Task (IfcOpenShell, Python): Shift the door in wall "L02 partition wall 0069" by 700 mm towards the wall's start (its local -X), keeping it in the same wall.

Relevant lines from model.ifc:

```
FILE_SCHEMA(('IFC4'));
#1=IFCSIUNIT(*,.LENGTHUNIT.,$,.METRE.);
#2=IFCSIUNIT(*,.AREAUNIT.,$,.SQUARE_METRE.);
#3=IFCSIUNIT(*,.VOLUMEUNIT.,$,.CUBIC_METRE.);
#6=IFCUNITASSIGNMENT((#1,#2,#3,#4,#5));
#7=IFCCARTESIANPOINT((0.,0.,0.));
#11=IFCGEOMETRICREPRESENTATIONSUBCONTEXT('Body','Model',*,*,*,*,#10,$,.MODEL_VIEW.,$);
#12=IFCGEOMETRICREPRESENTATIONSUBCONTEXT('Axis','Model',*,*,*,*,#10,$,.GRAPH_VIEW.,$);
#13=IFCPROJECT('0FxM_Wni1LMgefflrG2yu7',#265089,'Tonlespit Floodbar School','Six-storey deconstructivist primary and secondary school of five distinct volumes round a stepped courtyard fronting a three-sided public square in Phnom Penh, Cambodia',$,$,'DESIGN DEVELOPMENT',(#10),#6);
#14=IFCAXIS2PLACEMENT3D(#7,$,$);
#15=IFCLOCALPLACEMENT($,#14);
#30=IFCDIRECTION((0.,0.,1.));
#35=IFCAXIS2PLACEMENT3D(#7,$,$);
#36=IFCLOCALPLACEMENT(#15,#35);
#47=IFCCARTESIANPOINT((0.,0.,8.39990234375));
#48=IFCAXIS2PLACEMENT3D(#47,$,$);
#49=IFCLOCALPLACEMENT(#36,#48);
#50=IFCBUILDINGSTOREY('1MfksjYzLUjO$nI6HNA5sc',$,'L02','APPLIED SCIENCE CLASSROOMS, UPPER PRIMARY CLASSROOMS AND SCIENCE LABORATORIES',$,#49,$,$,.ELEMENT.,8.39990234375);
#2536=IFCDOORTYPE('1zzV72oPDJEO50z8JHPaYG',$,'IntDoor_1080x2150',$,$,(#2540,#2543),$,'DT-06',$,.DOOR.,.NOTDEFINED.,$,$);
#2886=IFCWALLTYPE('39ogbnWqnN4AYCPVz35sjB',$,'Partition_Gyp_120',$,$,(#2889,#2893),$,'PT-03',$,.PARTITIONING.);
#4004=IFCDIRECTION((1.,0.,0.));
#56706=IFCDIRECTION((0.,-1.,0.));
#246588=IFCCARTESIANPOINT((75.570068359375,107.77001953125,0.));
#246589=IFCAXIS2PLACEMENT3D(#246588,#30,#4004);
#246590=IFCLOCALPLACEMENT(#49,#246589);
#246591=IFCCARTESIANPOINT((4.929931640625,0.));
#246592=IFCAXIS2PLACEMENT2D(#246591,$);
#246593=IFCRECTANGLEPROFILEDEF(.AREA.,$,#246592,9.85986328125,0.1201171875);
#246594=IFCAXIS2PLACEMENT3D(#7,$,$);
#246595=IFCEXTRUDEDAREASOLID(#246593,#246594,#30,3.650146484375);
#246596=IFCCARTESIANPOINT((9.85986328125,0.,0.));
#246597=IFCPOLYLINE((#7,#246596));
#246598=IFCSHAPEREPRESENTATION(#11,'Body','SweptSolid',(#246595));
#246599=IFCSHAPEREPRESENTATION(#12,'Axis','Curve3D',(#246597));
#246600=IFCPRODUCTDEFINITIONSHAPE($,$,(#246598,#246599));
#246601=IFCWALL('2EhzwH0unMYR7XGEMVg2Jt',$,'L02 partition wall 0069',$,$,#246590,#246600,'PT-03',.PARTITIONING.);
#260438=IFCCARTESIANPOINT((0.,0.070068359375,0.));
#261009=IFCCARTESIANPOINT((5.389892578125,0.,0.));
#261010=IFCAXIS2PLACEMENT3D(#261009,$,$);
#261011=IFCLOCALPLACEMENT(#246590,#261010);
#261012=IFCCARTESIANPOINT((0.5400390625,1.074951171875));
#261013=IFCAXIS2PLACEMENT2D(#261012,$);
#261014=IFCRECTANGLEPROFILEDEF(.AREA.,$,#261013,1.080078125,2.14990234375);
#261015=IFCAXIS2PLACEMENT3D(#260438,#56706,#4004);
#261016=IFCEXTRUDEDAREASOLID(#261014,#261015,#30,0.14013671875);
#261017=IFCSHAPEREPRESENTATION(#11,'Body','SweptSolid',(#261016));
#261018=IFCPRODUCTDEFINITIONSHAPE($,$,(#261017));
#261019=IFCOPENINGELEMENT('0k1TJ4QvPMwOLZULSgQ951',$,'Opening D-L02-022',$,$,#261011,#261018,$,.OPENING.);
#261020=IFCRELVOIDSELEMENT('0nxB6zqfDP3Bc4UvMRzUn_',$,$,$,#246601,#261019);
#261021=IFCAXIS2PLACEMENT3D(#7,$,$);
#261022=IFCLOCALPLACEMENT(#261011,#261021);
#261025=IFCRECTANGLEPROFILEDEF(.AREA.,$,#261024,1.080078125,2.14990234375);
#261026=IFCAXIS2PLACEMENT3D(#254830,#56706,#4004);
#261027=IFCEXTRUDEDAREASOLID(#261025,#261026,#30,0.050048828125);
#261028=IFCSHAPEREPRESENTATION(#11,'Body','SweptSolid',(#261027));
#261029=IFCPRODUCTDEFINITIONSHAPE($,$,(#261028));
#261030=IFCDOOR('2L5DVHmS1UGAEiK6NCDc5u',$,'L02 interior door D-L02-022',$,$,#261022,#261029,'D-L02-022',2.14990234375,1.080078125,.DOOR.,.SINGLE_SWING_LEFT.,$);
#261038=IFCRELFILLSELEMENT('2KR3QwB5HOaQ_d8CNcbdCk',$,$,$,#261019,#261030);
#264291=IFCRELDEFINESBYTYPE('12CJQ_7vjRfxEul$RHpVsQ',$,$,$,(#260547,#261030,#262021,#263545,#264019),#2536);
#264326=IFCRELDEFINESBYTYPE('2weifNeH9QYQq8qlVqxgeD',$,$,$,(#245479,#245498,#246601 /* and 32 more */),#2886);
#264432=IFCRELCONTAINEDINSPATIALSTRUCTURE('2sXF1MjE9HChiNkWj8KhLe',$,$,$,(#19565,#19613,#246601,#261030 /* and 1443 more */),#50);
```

```python
import ifcopenshell
import ifcopenshell.api.geometry
import ifcopenshell.util.placement
import ifcopenshell.util.unit

model = ifcopenshell.open("model.ifc")
unit_scale = ifcopenshell.util.unit.calculate_unit_scale(model)

door = model.by_guid("2L5DVHmS1UGAEiK6NCDc5u")
opening = door.FillsVoids[0].RelatingOpeningElement
wall = opening.VoidsElements[0].RelatingBuildingElement

wall_matrix = ifcopenshell.util.placement.get_local_placement(wall.ObjectPlacement)
shift = wall_matrix[:3, 0] * -0.7 / unit_scale
before = ifcopenshell.util.placement.get_local_placement(door.ObjectPlacement)[:3, 3].copy()

# The door is placed relative to its opening, so it follows when the opening moves.
matrix = ifcopenshell.util.placement.get_local_placement(opening.ObjectPlacement)
matrix[:3, 3] += shift
ifcopenshell.api.geometry.edit_object_placement(
    model, product=opening, matrix=matrix, is_si=False, should_transform_children=True
)

after = ifcopenshell.util.placement.get_local_placement(door.ObjectPlacement)[:3, 3]
print("door moved by", (after - before).round(3) + 0.0)

model.write("model_updated.ifc")
```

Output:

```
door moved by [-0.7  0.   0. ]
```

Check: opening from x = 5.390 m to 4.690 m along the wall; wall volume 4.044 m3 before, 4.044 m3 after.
